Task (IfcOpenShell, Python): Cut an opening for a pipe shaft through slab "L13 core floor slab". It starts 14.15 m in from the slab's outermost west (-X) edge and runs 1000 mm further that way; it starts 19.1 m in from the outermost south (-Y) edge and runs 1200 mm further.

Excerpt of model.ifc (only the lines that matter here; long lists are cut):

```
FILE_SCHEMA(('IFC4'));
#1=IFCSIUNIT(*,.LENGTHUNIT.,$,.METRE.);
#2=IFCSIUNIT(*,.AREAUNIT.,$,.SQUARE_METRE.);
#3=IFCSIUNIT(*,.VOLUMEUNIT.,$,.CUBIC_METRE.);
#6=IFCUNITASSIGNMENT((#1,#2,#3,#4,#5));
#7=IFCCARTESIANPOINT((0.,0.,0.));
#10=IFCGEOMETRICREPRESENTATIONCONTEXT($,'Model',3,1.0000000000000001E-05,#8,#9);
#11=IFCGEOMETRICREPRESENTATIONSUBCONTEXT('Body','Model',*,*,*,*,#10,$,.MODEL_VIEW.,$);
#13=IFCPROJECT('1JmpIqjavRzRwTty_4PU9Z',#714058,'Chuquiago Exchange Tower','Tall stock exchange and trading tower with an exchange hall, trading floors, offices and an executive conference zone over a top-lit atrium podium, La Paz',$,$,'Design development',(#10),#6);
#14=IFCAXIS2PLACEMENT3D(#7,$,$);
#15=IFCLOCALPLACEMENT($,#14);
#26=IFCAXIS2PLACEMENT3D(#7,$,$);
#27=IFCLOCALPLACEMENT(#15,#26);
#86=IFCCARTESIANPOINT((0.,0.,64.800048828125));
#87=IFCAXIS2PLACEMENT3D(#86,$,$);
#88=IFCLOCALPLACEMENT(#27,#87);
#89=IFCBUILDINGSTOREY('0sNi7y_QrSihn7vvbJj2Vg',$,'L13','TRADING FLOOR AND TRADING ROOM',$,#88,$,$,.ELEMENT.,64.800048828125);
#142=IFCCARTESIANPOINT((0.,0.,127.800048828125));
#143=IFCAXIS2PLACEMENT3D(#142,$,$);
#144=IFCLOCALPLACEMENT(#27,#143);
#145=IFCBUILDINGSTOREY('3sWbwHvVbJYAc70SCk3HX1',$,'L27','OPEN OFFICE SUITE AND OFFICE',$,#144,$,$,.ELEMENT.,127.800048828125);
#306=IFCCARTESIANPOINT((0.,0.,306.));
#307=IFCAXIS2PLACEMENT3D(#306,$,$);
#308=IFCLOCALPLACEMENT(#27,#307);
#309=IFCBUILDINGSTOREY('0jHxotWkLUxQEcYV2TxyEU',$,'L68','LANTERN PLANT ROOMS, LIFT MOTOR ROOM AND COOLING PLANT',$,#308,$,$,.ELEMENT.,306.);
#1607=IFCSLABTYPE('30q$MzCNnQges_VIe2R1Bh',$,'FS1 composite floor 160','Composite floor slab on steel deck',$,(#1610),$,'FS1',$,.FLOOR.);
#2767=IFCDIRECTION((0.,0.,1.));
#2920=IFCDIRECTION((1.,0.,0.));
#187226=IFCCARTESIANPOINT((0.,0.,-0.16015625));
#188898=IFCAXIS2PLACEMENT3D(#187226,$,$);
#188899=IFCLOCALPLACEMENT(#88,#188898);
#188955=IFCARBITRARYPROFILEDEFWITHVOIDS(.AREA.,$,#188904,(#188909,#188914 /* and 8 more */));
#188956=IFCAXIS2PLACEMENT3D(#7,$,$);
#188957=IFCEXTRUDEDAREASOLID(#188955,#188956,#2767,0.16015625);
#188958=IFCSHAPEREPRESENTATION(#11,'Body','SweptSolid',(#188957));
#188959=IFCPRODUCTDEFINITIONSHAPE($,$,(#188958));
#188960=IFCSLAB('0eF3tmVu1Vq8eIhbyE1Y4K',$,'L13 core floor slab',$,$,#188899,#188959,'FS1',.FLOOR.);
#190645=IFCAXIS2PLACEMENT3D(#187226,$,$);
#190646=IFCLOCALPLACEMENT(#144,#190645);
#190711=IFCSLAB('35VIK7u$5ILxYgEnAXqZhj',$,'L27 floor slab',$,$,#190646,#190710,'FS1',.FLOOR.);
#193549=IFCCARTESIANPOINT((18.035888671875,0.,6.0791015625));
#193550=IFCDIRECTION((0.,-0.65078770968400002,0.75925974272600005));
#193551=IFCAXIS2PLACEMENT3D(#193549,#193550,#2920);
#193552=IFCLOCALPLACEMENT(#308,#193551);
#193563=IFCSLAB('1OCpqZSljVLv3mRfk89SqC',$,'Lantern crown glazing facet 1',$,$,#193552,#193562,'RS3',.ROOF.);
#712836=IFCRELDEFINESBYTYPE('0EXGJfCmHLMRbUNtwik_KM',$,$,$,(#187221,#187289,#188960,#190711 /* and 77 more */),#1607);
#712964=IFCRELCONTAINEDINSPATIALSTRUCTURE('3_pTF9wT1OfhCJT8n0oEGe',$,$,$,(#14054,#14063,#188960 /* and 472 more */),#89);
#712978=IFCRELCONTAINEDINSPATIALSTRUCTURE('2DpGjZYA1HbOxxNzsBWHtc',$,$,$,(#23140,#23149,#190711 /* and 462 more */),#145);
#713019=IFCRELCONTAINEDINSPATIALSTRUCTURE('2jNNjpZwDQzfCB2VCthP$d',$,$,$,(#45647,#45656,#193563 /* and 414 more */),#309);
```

```python
import numpy as np
import ifcopenshell
import ifcopenshell.api.feature
import ifcopenshell.api.geometry
import ifcopenshell.api.root
import ifcopenshell.geom
import ifcopenshell.util.placement
import ifcopenshell.util.representation
import ifcopenshell.util.shape
import ifcopenshell.util.unit

model = ifcopenshell.open("model.ifc")
unit_scale = ifcopenshell.util.unit.calculate_unit_scale(model)
settings = ifcopenshell.geom.settings()


def volume(element):
    """Net volume in cubic metres, openings subtracted."""
    shape = ifcopenshell.geom.create_shape(settings, element)
    return ifcopenshell.util.shape.get_volume(shape.geometry)


slab = model.by_guid("0eF3tmVu1Vq8eIhbyE1Y4K")
before = volume(slab)

# Extent in the slab's own axes, in metres. The edges named are its -X and -Y sides.
slab_shape = ifcopenshell.geom.create_shape(settings, slab)
vertices = ifcopenshell.util.shape.get_vertices(slab_shape.geometry)
x_min, y_min, bottom = vertices.min(axis=0)
top = vertices[:, 2].max()

opening = ifcopenshell.api.root.create_entity(model, ifc_class="IfcOpeningElement", name="Pipe shaft opening", predefined_type="OPENING")
context = ifcopenshell.util.representation.get_context(model, "Model", "Body", "MODEL_VIEW")
width, depth = 1, 1.2
outline = [(0.0, 0.0), (width, 0.0), (width, depth), (0.0, depth), (0.0, 0.0)]
# Overshoot both faces by 50 mm so the cut is clean.
shape = ifcopenshell.api.geometry.add_slab_representation(
    model, context=context, depth=top - bottom + 0.1, polyline=outline
)
ifcopenshell.api.geometry.assign_representation(model, product=opening, representation=shape)

matrix = ifcopenshell.util.placement.get_local_placement(slab.ObjectPlacement)
matrix[:, 3] = matrix @ np.append(np.array([x_min + 14.15, y_min + 19.1, bottom - 0.05]) / unit_scale, 1.0)
ifcopenshell.api.geometry.edit_object_placement(model, product=opening, matrix=matrix, is_si=False)
ifcopenshell.api.feature.add_feature(model, feature=opening, element=slab)

after = volume(slab)

print(f"slab volume {before:.3f} -> {after:.3f} m3")

model.write("model_edited.ifc")
```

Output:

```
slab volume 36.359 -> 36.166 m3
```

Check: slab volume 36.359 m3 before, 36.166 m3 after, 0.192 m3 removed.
